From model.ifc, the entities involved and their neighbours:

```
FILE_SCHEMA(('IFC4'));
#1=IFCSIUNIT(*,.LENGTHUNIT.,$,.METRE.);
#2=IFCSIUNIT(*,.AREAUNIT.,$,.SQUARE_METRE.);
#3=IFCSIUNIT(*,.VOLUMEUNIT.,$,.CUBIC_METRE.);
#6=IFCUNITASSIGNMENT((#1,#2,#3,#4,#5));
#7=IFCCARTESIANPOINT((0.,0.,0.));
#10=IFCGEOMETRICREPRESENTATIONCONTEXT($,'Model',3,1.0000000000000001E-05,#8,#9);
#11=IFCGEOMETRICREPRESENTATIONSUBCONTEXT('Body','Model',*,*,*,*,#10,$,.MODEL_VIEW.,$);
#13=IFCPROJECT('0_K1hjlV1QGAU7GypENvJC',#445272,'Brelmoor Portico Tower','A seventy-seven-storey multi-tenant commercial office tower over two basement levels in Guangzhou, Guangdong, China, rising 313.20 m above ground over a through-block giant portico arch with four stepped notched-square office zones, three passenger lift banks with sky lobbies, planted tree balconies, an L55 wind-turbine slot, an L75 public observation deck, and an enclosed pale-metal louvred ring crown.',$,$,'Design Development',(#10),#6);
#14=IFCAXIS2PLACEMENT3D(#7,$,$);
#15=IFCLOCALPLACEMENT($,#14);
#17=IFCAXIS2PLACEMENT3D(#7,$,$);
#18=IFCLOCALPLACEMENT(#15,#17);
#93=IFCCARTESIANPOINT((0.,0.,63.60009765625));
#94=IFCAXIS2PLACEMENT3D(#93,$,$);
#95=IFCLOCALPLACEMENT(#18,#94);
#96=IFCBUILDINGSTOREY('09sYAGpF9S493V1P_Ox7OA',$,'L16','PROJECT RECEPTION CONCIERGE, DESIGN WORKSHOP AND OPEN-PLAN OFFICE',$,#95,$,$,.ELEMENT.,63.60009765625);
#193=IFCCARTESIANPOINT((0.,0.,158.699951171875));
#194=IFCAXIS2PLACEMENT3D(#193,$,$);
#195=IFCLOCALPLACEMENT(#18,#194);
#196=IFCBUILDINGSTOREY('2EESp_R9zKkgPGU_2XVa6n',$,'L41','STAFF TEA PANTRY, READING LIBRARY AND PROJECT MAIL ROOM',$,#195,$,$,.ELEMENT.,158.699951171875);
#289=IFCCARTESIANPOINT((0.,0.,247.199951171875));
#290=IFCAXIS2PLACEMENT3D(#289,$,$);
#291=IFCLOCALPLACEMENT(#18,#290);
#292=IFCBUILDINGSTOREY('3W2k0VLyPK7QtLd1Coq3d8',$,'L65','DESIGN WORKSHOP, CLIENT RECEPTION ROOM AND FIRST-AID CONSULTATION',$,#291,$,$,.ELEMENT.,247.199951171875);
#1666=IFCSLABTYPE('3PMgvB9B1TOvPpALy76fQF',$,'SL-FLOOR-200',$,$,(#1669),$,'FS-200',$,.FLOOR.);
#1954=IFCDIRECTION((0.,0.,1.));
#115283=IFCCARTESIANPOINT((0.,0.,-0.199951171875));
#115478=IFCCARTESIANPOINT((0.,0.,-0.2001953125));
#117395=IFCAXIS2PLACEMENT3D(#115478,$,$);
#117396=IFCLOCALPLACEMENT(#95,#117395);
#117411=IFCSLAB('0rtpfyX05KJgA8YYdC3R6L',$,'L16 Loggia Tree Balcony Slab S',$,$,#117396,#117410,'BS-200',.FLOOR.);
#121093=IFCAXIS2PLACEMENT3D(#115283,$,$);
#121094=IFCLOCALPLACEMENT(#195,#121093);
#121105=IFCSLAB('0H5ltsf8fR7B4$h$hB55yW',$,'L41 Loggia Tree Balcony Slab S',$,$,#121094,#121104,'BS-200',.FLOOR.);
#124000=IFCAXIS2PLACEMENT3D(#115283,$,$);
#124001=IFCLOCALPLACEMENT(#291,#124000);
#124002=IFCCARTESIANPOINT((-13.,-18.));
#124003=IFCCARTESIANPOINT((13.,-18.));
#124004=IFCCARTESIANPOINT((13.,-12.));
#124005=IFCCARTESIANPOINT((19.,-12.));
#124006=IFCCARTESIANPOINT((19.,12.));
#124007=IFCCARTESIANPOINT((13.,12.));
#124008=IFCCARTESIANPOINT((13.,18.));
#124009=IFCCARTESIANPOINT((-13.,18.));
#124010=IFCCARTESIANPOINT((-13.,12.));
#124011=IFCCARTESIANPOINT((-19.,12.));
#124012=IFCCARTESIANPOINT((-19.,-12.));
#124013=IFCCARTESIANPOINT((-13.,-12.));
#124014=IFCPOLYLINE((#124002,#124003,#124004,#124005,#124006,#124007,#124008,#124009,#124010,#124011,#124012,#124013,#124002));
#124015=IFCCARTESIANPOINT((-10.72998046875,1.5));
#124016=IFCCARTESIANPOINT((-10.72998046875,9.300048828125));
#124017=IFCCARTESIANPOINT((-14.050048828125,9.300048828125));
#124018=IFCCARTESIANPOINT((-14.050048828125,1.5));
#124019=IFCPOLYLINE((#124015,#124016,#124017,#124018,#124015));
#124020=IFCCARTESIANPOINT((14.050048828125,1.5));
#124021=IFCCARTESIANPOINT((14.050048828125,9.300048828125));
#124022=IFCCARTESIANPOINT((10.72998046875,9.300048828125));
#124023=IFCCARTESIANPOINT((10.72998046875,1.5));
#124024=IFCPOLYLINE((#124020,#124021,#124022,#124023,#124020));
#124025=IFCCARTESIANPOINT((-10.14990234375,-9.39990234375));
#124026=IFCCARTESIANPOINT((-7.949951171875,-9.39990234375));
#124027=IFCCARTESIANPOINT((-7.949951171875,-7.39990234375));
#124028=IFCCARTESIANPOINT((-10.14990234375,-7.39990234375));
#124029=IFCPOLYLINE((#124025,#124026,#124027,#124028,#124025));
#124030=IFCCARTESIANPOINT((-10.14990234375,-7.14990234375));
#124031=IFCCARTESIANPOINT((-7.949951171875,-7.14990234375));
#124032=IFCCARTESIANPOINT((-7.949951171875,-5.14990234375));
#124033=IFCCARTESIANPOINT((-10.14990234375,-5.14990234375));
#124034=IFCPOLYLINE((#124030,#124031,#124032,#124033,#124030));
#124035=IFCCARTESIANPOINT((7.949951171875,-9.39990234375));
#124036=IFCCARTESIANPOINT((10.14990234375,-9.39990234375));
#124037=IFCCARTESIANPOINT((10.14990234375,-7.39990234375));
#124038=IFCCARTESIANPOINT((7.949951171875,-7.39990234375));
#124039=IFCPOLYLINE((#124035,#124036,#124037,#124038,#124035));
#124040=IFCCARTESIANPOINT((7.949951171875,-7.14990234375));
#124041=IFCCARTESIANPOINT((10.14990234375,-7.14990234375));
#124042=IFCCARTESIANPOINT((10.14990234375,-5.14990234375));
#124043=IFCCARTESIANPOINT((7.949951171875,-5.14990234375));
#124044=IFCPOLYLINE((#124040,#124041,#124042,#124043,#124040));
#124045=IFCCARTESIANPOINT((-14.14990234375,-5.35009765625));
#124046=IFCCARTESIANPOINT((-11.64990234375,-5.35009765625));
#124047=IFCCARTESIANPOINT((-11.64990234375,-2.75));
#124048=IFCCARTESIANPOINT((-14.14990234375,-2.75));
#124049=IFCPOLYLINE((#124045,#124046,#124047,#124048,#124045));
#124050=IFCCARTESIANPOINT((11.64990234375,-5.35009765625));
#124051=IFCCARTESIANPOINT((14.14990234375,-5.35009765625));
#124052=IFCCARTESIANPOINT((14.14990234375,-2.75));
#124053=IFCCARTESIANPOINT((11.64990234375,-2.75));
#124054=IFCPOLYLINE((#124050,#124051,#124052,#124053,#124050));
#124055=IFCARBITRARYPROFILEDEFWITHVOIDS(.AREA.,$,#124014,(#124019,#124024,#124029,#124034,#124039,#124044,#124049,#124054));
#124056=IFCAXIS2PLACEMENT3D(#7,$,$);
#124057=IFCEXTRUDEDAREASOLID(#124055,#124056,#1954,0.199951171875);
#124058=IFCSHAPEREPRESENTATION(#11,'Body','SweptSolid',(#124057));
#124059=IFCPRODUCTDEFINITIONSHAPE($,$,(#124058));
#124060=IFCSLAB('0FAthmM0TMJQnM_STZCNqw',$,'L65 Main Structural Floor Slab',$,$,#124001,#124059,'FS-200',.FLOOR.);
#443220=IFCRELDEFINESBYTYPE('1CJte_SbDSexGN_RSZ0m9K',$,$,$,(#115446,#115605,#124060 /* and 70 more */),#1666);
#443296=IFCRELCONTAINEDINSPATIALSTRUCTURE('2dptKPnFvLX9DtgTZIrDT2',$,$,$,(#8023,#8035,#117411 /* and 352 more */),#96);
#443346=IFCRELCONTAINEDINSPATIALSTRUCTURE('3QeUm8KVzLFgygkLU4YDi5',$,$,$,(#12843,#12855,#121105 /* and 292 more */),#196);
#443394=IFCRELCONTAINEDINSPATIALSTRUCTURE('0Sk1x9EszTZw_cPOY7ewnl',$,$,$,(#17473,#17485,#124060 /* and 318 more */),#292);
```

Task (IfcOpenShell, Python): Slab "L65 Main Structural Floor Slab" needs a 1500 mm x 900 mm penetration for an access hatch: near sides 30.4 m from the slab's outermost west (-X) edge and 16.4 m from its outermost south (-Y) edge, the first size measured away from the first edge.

```python
import numpy as np
import ifcopenshell
import ifcopenshell.api.feature
import ifcopenshell.api.geometry
import ifcopenshell.api.root
import ifcopenshell.geom
import ifcopenshell.util.placement
import ifcopenshell.util.representation
import ifcopenshell.util.shape
import ifcopenshell.util.unit

model = ifcopenshell.open("model.ifc")
unit_scale = ifcopenshell.util.unit.calculate_unit_scale(model)
settings = ifcopenshell.geom.settings()


def volume(element):
    """Net volume in cubic metres, openings subtracted."""
    shape = ifcopenshell.geom.create_shape(settings, element)
    return ifcopenshell.util.shape.get_volume(shape.geometry)


slab = model.by_guid("0FAthmM0TMJQnM_STZCNqw")
before = volume(slab)

# Extent in the slab's own axes, in metres. The edges named are its -X and -Y sides.
slab_shape = ifcopenshell.geom.create_shape(settings, slab)
vertices = ifcopenshell.util.shape.get_vertices(slab_shape.geometry)
x_min, y_min, bottom = vertices.min(axis=0)
top = vertices[:, 2].max()

opening = ifcopenshell.api.root.create_entity(model, ifc_class="IfcOpeningElement", name="Access hatch opening", predefined_type="OPENING")
context = ifcopenshell.util.representation.get_context(model, "Model", "Body", "MODEL_VIEW")
width, depth = 1.5, 0.9
outline = [(0.0, 0.0), (width, 0.0), (width, depth), (0.0, depth), (0.0, 0.0)]
# Overshoot both faces by 50 mm so the cut is clean.
shape = ifcopenshell.api.geometry.add_slab_representation(
    model, context=context, depth=top - bottom + 0.1, polyline=outline
)
ifcopenshell.api.geometry.assign_representation(model, product=opening, representation=shape)

matrix = ifcopenshell.util.placement.get_local_placement(slab.ObjectPlacement)
matrix[:, 3] = matrix @ np.append(np.array([x_min + 30.4, y_min + 16.4, bottom - 0.05]) / unit_scale, 1.0)
ifcopenshell.api.geometry.edit_object_placement(model, product=opening, matrix=matrix, is_si=False)
ifcopenshell.api.feature.add_feature(model, feature=opening, element=slab)

after = volume(slab)

print(f"slab volume {before:.3f} -> {after:.3f} m3")

model.write("model_v2.ifc")
```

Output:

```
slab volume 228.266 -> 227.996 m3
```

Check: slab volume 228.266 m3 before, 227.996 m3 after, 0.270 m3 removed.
